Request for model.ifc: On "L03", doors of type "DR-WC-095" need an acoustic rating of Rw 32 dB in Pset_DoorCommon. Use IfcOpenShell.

First a look at what the model holds.

```python
import ifcopenshell
import ifcopenshell.util.element

model = ifcopenshell.open("model.ifc")
print(model.schema)
storey = next(s for s in model.by_type("IfcBuildingStorey") if s.Name == "L03")
doors = [e for e in ifcopenshell.util.element.get_decomposition(storey) if e.is_a("IfcDoor")]
seen = {}
for e in doors:
    element_type = ifcopenshell.util.element.get_type(e)
    key = (element_type.Name if element_type != e and element_type else None, ifcopenshell.util.element.get_pset(e, "Pset_DoorCommon", "AcousticRating"))
    seen[key] = seen.get(key, 0) + 1
for (name, value), count in sorted(seen.items(), key=str):
    print(count, "x", name, "|", value)
```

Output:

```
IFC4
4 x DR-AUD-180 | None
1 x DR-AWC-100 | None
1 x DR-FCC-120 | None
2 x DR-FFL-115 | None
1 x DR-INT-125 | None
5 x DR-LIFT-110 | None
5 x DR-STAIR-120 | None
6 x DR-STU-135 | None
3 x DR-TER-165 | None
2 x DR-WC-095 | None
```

```python
import ifcopenshell
import ifcopenshell.api.pset
import ifcopenshell.util.element

model = ifcopenshell.open("model.ifc")

storey = next(s for s in model.by_type("IfcBuildingStorey") if s.Name == "L03")
doors = [e for e in ifcopenshell.util.element.get_decomposition(storey) if e.is_a("IfcDoor")]

count = 0
for e in doors:
    element_type = ifcopenshell.util.element.get_type(e)
    if element_type in (None, e) or element_type.Name != "DR-WC-095":
        continue
    # add_pset returns the element's existing set when there is one.
    pset = ifcopenshell.api.pset.add_pset(model, product=e, name="Pset_DoorCommon")
    ifcopenshell.api.pset.edit_pset(model, pset=pset, properties={"AcousticRating": "Rw 32 dB"})
    count += 1

print(count, "doors updated")

model.write("model_edited.ifc")
```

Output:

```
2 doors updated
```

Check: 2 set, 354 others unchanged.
